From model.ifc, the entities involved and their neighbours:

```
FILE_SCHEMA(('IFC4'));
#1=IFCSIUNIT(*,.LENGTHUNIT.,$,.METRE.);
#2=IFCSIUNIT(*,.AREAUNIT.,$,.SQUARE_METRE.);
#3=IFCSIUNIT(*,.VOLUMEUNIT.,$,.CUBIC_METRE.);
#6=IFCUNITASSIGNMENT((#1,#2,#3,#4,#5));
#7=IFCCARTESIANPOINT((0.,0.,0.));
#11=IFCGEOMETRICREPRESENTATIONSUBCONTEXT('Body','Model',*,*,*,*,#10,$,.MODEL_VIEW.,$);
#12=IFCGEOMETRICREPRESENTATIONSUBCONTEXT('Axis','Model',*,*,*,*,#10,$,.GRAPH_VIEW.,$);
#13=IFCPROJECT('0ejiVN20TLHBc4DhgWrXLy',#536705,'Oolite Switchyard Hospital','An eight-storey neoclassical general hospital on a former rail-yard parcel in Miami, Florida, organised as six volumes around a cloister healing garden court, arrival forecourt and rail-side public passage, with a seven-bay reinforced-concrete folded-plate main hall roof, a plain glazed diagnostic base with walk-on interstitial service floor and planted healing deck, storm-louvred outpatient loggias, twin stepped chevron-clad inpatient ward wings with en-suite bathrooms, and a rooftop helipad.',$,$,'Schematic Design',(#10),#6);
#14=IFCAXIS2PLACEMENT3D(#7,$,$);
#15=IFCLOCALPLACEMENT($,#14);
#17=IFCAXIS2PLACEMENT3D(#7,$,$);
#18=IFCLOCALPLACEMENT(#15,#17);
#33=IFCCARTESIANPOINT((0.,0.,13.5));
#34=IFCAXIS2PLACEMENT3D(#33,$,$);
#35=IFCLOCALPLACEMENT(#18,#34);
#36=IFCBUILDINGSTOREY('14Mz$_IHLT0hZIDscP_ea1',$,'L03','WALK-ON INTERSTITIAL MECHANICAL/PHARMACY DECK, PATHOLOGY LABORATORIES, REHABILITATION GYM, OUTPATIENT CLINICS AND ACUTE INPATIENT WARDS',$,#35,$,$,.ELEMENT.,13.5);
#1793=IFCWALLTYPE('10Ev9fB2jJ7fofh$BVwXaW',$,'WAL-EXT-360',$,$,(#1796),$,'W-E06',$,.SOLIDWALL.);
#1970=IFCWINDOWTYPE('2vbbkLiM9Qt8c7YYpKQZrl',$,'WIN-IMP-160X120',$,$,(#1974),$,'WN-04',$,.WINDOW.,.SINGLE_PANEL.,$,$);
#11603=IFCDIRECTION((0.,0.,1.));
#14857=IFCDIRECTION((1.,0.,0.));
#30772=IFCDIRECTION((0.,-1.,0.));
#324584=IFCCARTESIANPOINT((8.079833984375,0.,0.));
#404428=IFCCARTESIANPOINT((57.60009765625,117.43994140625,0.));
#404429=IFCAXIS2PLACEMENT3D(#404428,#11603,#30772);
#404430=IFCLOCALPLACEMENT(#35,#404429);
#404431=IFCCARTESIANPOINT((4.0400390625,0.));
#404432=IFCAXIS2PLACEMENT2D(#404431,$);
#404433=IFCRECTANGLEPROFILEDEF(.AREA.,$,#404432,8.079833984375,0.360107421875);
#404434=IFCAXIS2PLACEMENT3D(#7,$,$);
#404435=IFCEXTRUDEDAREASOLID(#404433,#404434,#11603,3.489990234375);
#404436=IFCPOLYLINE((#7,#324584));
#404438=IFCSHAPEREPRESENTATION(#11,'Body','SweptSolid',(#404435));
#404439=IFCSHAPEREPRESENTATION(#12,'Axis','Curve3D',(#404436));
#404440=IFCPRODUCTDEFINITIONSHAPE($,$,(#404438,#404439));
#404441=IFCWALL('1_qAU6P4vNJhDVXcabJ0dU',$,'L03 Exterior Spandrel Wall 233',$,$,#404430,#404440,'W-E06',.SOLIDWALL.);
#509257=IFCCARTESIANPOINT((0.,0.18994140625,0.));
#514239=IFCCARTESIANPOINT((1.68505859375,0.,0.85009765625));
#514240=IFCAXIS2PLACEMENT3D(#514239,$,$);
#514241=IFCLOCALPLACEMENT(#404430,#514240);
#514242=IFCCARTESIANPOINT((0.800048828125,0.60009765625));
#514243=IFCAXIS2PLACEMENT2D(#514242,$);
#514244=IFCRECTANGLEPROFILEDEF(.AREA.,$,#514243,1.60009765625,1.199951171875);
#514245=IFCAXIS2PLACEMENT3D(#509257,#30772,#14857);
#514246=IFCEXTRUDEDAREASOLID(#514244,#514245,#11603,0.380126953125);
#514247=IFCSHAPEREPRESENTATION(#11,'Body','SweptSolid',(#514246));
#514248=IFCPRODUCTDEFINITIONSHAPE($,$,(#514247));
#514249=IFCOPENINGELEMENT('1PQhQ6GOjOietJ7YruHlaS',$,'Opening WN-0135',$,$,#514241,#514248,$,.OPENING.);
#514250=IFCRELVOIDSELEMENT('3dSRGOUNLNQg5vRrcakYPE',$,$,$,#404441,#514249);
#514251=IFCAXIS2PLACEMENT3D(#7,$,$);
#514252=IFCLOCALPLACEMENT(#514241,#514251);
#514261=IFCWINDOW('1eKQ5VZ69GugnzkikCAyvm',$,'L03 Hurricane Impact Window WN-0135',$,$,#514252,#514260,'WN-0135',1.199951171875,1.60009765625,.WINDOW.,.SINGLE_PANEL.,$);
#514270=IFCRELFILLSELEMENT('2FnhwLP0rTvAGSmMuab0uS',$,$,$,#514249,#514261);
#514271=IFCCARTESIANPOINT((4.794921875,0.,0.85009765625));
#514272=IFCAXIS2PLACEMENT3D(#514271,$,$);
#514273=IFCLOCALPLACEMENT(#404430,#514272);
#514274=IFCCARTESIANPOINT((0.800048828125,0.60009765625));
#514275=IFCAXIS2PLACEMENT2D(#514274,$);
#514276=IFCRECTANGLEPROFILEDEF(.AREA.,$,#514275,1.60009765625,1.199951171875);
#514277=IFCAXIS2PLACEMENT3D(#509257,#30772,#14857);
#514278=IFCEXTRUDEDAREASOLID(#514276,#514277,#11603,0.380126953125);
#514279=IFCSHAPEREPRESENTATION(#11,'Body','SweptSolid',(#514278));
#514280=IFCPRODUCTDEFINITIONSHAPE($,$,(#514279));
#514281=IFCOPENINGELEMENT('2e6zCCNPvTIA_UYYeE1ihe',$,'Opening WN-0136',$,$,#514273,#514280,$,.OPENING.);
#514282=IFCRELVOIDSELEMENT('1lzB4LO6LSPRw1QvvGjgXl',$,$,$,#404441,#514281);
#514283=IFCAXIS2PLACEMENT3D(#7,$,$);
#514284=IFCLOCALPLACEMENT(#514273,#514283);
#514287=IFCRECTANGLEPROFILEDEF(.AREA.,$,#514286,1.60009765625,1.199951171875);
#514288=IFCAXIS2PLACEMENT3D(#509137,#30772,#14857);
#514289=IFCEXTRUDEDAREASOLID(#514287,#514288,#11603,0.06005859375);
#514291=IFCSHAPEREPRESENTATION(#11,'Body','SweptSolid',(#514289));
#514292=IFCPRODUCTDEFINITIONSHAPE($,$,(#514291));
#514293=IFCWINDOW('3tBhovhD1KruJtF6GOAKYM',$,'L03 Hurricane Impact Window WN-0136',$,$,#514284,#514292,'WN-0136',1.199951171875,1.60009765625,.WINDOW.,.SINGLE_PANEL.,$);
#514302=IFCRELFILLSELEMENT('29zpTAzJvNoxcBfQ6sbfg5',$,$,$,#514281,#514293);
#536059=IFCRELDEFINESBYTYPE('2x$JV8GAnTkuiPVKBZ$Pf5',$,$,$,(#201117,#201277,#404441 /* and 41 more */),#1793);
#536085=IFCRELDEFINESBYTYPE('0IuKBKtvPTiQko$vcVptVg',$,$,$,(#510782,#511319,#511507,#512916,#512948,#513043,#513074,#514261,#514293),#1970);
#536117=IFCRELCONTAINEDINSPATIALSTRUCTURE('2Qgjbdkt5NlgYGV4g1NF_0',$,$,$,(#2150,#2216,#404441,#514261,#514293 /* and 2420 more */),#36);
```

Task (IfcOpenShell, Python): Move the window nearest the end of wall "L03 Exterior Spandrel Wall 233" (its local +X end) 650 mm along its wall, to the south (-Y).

```python
import ifcopenshell
import ifcopenshell.api.geometry
import ifcopenshell.util.placement
import ifcopenshell.util.unit

model = ifcopenshell.open("model.ifc")
unit_scale = ifcopenshell.util.unit.calculate_unit_scale(model)

window = model.by_guid("3tBhovhD1KruJtF6GOAKYM")
opening = window.FillsVoids[0].RelatingOpeningElement
wall = opening.VoidsElements[0].RelatingBuildingElement

wall_matrix = ifcopenshell.util.placement.get_local_placement(wall.ObjectPlacement)
shift = wall_matrix[:3, 0] * 0.65 / unit_scale
before = ifcopenshell.util.placement.get_local_placement(window.ObjectPlacement)[:3, 3].copy()

# The window is placed relative to its opening, so it follows when the opening moves.
matrix = ifcopenshell.util.placement.get_local_placement(opening.ObjectPlacement)
matrix[:3, 3] += shift
ifcopenshell.api.geometry.edit_object_placement(
    model, product=opening, matrix=matrix, is_si=False, should_transform_children=True
)

after = ifcopenshell.util.placement.get_local_placement(window.ObjectPlacement)[:3, 3]
print("window moved by", (after - before).round(3) + 0.0)

model.write("model_v2.ifc")
```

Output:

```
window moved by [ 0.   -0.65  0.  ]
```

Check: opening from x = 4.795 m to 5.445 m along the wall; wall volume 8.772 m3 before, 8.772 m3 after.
